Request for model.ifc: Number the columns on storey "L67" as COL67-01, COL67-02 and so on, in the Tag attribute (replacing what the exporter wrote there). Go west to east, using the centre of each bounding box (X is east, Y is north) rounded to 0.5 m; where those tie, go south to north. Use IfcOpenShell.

First a look at what the model holds.

```python
import ifcopenshell
import ifcopenshell.util.element
import ifcopenshell.util.placement

model = ifcopenshell.open("model.ifc")
print(model.schema)
storey = next(s for s in model.by_type("IfcBuildingStorey") if s.Name == "L67")
columns = [e for e in ifcopenshell.util.element.get_decomposition(storey) if e.is_a("IfcColumn")]
for e in sorted(columns, key=lambda e: e.id()):
    origin = ifcopenshell.util.placement.get_local_placement(e.ObjectPlacement)[:3, 3]
    print(e.id(), e.Tag, e.Name, origin.round(2) + 0.0, sep=" | ")
```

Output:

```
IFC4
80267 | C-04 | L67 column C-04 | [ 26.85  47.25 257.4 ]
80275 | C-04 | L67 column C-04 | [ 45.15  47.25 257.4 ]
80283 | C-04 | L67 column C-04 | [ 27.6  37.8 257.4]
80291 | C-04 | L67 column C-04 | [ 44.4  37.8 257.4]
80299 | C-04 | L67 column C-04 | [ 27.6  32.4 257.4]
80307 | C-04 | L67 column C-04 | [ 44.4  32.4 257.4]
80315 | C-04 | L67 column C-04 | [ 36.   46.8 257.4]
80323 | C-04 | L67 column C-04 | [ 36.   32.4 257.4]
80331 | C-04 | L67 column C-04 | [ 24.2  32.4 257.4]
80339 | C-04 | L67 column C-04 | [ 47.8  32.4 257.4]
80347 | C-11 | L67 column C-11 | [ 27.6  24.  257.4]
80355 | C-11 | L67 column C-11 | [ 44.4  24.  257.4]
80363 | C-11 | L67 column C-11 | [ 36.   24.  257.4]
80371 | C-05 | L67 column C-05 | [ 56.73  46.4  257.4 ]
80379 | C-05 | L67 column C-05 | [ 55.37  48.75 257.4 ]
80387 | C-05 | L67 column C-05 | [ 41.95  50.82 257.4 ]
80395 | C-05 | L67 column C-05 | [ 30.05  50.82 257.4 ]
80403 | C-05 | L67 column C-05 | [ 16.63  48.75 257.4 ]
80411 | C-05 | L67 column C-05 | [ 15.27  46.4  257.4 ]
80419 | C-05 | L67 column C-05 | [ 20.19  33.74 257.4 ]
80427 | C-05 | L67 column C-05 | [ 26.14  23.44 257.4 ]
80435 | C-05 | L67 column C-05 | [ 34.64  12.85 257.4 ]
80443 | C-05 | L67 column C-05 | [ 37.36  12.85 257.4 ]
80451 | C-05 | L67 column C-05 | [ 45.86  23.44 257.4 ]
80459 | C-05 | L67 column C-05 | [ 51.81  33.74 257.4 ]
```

```python
import ifcopenshell
import ifcopenshell.geom
import ifcopenshell.util.element
import ifcopenshell.util.shape

model = ifcopenshell.open("model.ifc")
settings = ifcopenshell.geom.settings()
settings.set("use-world-coords", True)


def centre(element):
    shape = ifcopenshell.geom.create_shape(settings, element)
    return ifcopenshell.util.shape.get_bbox_centroid(shape.geometry)


storey = next(s for s in model.by_type("IfcBuildingStorey") if s.Name == "L67")
columns = [e for e in ifcopenshell.util.element.get_decomposition(storey) if e.is_a("IfcColumn")]

# Insertion points can sit at a corner or the storey origin, so sort by the geometry (in metres).
centres = {e: centre(e) for e in columns}
columns.sort(key=lambda e: (round(centres[e][0] / 0.5), centres[e][1]))

for i, e in enumerate(columns, start=1):
    number = f"COL67-{i:02d}"
    e.Tag = number
    print(e.id(), number)

model.write("model_updated.ifc")
```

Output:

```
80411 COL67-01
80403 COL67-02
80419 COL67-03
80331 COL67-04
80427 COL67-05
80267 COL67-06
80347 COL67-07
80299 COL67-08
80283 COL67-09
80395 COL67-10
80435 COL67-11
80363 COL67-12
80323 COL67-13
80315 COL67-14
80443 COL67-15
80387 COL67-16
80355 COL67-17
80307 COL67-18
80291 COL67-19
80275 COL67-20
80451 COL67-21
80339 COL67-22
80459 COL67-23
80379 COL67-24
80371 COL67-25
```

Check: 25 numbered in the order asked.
